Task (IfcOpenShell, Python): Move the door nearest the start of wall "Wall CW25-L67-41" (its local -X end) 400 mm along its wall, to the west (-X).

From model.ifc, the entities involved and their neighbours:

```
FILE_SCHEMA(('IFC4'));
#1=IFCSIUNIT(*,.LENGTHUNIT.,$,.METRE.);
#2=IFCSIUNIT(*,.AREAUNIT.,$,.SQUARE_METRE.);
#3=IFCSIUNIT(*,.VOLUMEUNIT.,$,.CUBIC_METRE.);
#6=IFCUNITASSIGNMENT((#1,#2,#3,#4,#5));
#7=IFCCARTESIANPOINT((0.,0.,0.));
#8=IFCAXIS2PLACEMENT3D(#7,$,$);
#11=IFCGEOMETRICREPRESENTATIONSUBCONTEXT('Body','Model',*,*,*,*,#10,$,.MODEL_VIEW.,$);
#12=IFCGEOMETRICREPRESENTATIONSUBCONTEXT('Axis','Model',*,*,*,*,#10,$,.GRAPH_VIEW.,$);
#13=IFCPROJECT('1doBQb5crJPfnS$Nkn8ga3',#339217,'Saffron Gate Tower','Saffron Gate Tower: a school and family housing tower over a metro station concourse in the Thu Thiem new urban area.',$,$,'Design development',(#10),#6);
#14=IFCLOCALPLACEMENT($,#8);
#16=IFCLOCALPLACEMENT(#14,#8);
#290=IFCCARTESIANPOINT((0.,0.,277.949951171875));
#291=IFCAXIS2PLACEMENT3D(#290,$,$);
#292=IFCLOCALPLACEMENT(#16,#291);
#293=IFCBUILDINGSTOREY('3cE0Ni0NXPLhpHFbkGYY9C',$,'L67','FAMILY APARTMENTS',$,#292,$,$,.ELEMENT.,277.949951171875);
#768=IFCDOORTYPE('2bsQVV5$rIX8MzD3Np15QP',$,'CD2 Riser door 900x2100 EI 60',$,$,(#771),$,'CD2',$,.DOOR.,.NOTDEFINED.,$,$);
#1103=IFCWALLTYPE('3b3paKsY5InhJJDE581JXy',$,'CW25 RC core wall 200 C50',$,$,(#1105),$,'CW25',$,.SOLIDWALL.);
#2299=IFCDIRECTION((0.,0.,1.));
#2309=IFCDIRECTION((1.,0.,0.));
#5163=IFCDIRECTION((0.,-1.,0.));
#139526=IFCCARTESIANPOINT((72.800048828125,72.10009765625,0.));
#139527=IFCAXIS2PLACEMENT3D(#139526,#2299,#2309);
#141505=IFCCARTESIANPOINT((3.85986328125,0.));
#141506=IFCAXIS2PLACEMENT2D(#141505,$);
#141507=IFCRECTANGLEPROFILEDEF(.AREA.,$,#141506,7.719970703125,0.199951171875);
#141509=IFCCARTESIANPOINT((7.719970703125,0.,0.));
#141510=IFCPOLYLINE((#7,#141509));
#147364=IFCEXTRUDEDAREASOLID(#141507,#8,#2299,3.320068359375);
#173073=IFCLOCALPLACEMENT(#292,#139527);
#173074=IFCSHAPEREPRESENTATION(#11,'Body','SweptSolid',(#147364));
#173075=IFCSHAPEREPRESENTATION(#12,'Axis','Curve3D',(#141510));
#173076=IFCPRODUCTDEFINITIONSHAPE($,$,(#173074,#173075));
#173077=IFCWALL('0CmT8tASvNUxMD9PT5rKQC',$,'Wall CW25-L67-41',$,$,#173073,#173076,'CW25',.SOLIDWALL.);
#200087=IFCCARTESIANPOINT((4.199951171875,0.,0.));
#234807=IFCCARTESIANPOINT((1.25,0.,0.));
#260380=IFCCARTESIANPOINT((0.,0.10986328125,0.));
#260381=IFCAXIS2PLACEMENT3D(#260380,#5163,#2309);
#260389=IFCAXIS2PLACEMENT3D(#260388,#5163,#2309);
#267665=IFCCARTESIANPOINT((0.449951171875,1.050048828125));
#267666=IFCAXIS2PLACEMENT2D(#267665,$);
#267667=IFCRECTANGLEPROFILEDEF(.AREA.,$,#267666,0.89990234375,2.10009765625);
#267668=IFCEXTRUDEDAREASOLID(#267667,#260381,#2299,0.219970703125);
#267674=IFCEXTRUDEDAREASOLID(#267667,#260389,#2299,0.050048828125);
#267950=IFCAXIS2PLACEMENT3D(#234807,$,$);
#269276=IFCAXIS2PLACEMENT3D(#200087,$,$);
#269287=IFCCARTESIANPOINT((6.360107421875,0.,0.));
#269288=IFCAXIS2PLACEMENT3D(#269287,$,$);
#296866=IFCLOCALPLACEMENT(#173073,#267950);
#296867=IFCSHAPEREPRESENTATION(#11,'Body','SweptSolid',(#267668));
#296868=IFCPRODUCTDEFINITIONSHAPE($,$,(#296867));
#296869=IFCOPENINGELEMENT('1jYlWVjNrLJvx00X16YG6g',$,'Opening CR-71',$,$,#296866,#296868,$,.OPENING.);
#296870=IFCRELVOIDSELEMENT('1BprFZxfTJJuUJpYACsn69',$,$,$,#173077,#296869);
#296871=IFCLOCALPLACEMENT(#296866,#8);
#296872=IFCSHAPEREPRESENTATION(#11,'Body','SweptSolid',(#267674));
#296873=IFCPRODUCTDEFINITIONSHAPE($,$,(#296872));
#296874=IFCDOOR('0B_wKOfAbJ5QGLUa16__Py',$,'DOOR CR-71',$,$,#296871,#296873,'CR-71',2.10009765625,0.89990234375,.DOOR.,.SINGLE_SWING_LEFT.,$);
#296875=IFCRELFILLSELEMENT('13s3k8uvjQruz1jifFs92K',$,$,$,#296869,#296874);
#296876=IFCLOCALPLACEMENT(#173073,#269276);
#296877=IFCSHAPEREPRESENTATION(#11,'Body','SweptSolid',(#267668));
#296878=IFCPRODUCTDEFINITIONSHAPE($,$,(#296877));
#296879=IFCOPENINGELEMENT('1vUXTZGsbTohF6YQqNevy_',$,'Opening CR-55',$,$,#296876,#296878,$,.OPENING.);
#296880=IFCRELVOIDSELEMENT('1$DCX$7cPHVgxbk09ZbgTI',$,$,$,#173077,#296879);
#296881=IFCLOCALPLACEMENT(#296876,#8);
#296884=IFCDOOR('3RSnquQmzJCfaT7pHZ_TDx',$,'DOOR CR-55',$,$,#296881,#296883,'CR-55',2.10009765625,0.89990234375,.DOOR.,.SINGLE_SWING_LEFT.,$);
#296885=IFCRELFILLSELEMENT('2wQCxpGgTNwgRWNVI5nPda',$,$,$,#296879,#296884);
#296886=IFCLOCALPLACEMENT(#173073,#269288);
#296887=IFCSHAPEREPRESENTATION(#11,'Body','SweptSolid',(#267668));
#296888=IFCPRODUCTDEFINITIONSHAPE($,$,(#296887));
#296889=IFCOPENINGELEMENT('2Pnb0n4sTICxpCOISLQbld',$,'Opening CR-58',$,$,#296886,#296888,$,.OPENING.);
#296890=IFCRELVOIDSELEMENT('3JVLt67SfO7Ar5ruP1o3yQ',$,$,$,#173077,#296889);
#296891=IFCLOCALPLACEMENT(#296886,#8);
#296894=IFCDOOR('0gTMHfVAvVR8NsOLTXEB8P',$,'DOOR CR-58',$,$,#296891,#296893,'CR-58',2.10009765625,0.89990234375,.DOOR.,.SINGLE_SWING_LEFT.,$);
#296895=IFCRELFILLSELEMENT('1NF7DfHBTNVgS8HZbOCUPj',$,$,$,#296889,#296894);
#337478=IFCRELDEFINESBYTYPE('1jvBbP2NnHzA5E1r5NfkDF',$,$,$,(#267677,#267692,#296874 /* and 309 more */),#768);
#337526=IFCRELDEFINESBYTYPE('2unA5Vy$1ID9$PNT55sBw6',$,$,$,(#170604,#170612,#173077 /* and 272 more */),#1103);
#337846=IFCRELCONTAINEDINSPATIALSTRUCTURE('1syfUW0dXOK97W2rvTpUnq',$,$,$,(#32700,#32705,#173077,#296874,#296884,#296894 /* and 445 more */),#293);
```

```python
import ifcopenshell
import ifcopenshell.api.geometry
import ifcopenshell.util.placement
import ifcopenshell.util.unit

model = ifcopenshell.open("model.ifc")
unit_scale = ifcopenshell.util.unit.calculate_unit_scale(model)

door = model.by_id(296874)
opening = door.FillsVoids[0].RelatingOpeningElement
wall = opening.VoidsElements[0].RelatingBuildingElement

wall_matrix = ifcopenshell.util.placement.get_local_placement(wall.ObjectPlacement)
shift = wall_matrix[:3, 0] * -0.4 / unit_scale
before = ifcopenshell.util.placement.get_local_placement(door.ObjectPlacement)[:3, 3].copy()

# The door is placed relative to its opening, so it follows when the opening moves.
matrix = ifcopenshell.util.placement.get_local_placement(opening.ObjectPlacement)
matrix[:3, 3] += shift
ifcopenshell.api.geometry.edit_object_placement(
    model, product=opening, matrix=matrix, is_si=False, should_transform_children=True
)

after = ifcopenshell.util.placement.get_local_placement(door.ObjectPlacement)[:3, 3]
print("door moved by", (after - before).round(3) + 0.0)

model.write("model_rev.ifc")
```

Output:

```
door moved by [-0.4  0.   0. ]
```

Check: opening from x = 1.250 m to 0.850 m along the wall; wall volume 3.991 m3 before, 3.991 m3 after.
